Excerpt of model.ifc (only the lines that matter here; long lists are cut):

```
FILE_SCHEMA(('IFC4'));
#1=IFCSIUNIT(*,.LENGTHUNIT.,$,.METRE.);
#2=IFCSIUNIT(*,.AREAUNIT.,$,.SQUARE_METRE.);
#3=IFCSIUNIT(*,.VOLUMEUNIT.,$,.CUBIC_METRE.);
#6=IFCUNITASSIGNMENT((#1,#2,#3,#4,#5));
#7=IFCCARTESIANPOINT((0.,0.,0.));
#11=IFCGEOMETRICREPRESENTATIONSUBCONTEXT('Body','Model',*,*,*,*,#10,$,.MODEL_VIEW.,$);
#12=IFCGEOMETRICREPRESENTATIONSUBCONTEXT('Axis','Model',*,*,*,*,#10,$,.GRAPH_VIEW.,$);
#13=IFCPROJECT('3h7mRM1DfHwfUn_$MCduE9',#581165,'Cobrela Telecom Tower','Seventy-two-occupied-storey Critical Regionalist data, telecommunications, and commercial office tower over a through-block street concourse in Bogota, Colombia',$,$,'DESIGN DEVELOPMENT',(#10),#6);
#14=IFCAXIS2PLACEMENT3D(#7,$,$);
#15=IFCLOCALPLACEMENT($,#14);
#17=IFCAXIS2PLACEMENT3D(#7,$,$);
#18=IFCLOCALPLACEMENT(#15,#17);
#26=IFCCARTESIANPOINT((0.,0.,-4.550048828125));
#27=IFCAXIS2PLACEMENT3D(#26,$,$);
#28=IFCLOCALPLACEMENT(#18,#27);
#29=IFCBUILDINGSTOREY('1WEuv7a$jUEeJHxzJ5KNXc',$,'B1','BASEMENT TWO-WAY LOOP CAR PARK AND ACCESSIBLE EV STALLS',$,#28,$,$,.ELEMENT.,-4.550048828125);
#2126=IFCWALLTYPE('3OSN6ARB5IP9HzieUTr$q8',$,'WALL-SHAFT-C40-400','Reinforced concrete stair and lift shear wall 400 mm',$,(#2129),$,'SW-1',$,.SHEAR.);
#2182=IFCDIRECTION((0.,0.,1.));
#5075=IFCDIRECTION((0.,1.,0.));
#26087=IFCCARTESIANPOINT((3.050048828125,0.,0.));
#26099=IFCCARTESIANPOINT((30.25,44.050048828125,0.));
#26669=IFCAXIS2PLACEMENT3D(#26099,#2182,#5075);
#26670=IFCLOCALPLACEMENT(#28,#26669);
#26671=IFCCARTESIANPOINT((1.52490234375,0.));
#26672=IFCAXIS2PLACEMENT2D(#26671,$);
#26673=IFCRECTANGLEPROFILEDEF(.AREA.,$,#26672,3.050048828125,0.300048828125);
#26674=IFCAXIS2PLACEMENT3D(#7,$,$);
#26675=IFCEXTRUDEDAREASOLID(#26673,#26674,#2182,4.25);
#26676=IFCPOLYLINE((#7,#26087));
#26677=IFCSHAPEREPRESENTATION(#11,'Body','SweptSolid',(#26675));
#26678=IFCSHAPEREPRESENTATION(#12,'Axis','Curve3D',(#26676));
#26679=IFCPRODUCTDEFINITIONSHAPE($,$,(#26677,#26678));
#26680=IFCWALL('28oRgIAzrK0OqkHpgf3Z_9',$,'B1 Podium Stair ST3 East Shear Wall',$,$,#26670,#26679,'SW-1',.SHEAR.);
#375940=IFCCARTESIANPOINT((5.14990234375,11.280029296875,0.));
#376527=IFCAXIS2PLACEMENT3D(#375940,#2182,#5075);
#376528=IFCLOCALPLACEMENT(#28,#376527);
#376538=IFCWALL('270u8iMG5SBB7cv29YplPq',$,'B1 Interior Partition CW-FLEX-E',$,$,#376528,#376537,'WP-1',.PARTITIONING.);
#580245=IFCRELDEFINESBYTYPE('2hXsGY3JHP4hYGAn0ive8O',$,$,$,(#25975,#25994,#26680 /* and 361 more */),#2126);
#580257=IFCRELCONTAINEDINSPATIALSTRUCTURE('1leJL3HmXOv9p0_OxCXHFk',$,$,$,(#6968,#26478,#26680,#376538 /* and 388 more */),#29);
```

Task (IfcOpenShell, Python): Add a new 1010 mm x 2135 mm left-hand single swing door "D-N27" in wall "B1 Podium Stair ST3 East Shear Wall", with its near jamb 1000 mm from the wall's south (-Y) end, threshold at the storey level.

```python
import numpy as np
import ifcopenshell
import ifcopenshell.api.feature
import ifcopenshell.api.geometry
import ifcopenshell.api.root
import ifcopenshell.api.spatial
import ifcopenshell.geom
import ifcopenshell.util.element
import ifcopenshell.util.placement
import ifcopenshell.util.representation
import ifcopenshell.util.shape
import ifcopenshell.util.unit

model = ifcopenshell.open("model.ifc")
unit_scale = ifcopenshell.util.unit.calculate_unit_scale(model)
settings = ifcopenshell.geom.settings()


def volume(element):
    """Net volume in cubic metres, openings subtracted."""
    shape = ifcopenshell.geom.create_shape(settings, element)
    return ifcopenshell.util.shape.get_volume(shape.geometry)


wall = model.by_guid("28oRgIAzrK0OqkHpgf3Z_9")
storey = ifcopenshell.util.element.get_container(wall, ifc_class="IfcBuildingStorey")
context = ifcopenshell.util.representation.get_context(model, "Model", "Body", "MODEL_VIEW")
before = volume(wall)

width, height, from_end, sill = 1.01, 2.135, 1, 0.0  # metres

# The wall runs along its own X axis, and the end named is its -X end.
wall_shape = ifcopenshell.geom.create_shape(settings, wall)
x, y, z = ifcopenshell.util.shape.get_vertices(wall_shape.geometry).T
start = x.min() + from_end
face, thickness = float(y.min()), float(y.max() - y.min())
wall_matrix = ifcopenshell.util.placement.get_local_placement(wall.ObjectPlacement)
level = ifcopenshell.util.placement.get_local_placement(storey.ObjectPlacement)[2, 3]


def in_wall(x, y):
    """Placement at x, y metres in the wall's axes, at sill height."""
    matrix = wall_matrix.copy()
    matrix[:, 3] = wall_matrix @ np.array([x / unit_scale, y / unit_scale, 0.0, 1.0])
    matrix[2, 3] = level + sill / unit_scale
    return matrix


# Opening: a box that overshoots both wall faces by 50 mm.
opening = ifcopenshell.api.root.create_entity(model, ifc_class="IfcOpeningElement", predefined_type="OPENING")
box = ifcopenshell.api.geometry.add_wall_representation(
    model, context=context, length=width, height=height, thickness=thickness + 0.1
)
ifcopenshell.api.geometry.assign_representation(model, product=opening, representation=box)
ifcopenshell.api.geometry.edit_object_placement(model, product=opening, matrix=in_wall(start, face - 0.05), is_si=False)
ifcopenshell.api.feature.add_feature(model, feature=opening, element=wall)

door = ifcopenshell.api.root.create_entity(model, ifc_class="IfcDoor", name="D-N27", predefined_type="DOOR")
door.OverallWidth, door.OverallHeight = width / unit_scale, height / unit_scale
door.OperationType = "SINGLE_SWING_LEFT"
body = ifcopenshell.api.geometry.add_door_representation(
    model,
    context=context,
    overall_width=door.OverallWidth,
    overall_height=door.OverallHeight,
    operation_type="SINGLE_SWING_LEFT",
    lining_properties={"LiningDepth": thickness / unit_scale, "ThresholdDepth": thickness / unit_scale},
)
ifcopenshell.api.geometry.assign_representation(model, product=door, representation=body)
ifcopenshell.api.spatial.assign_container(model, products=[door], relating_structure=storey)
ifcopenshell.api.feature.add_filling(model, opening=opening, element=door)

# The lining spans the wall, so the door starts at the wall face.
ifcopenshell.api.geometry.edit_object_placement(model, product=door, matrix=in_wall(start, face), is_si=False)

after = volume(wall)

print(f"wall volume {before:.3f} -> {after:.3f} m3")

model.write("model-out.ifc")
```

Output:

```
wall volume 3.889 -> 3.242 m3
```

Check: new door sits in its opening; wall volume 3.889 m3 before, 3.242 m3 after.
